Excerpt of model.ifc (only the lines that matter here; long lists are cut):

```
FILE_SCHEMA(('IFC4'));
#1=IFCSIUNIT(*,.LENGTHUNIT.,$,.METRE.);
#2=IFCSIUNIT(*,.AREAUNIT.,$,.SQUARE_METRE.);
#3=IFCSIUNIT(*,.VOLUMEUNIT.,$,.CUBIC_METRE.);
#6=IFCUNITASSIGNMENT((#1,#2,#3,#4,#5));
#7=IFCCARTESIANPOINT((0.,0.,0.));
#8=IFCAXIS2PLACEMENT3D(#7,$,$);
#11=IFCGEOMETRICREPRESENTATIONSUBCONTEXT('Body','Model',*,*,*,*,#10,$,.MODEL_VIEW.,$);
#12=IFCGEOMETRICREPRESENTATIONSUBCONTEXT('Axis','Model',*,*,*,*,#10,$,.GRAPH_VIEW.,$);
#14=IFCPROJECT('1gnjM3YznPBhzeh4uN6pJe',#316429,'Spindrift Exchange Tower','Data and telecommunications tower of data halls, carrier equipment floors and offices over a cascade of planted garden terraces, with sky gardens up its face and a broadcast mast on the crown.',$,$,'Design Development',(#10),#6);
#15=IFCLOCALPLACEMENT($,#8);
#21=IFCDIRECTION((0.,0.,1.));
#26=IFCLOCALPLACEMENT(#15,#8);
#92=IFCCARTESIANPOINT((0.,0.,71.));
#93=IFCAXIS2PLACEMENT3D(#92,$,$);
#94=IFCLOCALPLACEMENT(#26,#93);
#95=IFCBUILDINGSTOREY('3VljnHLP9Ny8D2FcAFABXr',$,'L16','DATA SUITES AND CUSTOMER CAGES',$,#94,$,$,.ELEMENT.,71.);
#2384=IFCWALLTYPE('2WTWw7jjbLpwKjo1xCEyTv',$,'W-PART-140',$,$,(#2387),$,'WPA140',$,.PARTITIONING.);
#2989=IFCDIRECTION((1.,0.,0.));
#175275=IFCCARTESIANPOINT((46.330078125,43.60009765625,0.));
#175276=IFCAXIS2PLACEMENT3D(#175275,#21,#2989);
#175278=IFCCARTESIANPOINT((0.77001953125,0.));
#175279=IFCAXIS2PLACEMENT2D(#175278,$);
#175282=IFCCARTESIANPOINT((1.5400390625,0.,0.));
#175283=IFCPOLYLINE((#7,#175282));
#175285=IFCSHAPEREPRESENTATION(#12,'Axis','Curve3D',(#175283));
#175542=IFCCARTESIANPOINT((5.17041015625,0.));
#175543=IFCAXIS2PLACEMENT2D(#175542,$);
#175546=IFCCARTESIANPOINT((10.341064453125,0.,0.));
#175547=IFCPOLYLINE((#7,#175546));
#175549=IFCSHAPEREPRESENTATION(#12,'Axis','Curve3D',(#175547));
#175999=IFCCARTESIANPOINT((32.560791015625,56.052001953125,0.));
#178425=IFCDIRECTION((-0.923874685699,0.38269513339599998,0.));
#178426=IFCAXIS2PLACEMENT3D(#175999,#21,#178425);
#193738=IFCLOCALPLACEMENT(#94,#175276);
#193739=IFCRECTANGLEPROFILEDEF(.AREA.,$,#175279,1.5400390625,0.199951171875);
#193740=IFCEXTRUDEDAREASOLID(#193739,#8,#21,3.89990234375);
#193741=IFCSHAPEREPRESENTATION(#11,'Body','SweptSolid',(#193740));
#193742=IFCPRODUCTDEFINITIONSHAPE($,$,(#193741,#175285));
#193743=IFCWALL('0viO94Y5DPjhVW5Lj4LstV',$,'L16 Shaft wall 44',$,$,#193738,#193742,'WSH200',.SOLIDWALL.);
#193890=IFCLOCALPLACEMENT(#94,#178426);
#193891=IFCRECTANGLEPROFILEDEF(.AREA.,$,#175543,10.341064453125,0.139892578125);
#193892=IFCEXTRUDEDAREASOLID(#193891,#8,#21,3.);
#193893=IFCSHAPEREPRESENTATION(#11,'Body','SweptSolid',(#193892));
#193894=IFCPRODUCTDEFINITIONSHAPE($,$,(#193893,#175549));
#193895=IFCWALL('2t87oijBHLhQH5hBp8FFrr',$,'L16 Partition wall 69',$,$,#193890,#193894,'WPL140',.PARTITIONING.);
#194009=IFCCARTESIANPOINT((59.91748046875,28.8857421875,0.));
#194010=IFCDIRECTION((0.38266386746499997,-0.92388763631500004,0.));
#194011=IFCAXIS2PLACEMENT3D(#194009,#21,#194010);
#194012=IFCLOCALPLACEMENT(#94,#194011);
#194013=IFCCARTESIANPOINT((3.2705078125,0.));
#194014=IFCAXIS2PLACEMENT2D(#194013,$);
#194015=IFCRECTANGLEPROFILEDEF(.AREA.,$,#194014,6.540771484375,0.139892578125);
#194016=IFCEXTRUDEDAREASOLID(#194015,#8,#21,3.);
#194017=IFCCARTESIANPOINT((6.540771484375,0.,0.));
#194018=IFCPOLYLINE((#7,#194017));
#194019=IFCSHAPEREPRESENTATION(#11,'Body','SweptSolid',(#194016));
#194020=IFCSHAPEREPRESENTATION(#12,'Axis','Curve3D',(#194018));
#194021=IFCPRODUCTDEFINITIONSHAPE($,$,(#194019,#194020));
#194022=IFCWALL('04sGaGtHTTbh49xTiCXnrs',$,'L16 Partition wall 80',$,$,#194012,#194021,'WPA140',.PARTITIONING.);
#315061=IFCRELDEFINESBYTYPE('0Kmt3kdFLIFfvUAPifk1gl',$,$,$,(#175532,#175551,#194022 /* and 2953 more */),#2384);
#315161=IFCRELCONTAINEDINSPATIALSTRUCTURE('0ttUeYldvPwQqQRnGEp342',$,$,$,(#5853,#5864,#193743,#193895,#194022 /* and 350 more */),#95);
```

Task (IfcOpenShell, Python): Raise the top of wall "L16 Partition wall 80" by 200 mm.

```python
import ifcopenshell
import ifcopenshell.geom
import ifcopenshell.util.representation
import ifcopenshell.util.shape
import ifcopenshell.util.unit

model = ifcopenshell.open("model.ifc")
unit_scale = ifcopenshell.util.unit.calculate_unit_scale(model)
settings = ifcopenshell.geom.settings()


def volume(element):
    """Net volume in cubic metres, openings subtracted."""
    shape = ifcopenshell.geom.create_shape(settings, element)
    return ifcopenshell.util.shape.get_volume(shape.geometry)


wall = model.by_id(194022)
before = volume(wall)

body = ifcopenshell.util.representation.get_representation(wall, "Model", "Body")
solid = body.Items[0]
old_height = solid.Depth
solid.Depth += 0.2 / unit_scale
after = volume(wall)

print(f"height {old_height:g} -> {solid.Depth:g}, volume {before:.3f} -> {after:.3f} m3")

model.write("model_rev.ifc")
```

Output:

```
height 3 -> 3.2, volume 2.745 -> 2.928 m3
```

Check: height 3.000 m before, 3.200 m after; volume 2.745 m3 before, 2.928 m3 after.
